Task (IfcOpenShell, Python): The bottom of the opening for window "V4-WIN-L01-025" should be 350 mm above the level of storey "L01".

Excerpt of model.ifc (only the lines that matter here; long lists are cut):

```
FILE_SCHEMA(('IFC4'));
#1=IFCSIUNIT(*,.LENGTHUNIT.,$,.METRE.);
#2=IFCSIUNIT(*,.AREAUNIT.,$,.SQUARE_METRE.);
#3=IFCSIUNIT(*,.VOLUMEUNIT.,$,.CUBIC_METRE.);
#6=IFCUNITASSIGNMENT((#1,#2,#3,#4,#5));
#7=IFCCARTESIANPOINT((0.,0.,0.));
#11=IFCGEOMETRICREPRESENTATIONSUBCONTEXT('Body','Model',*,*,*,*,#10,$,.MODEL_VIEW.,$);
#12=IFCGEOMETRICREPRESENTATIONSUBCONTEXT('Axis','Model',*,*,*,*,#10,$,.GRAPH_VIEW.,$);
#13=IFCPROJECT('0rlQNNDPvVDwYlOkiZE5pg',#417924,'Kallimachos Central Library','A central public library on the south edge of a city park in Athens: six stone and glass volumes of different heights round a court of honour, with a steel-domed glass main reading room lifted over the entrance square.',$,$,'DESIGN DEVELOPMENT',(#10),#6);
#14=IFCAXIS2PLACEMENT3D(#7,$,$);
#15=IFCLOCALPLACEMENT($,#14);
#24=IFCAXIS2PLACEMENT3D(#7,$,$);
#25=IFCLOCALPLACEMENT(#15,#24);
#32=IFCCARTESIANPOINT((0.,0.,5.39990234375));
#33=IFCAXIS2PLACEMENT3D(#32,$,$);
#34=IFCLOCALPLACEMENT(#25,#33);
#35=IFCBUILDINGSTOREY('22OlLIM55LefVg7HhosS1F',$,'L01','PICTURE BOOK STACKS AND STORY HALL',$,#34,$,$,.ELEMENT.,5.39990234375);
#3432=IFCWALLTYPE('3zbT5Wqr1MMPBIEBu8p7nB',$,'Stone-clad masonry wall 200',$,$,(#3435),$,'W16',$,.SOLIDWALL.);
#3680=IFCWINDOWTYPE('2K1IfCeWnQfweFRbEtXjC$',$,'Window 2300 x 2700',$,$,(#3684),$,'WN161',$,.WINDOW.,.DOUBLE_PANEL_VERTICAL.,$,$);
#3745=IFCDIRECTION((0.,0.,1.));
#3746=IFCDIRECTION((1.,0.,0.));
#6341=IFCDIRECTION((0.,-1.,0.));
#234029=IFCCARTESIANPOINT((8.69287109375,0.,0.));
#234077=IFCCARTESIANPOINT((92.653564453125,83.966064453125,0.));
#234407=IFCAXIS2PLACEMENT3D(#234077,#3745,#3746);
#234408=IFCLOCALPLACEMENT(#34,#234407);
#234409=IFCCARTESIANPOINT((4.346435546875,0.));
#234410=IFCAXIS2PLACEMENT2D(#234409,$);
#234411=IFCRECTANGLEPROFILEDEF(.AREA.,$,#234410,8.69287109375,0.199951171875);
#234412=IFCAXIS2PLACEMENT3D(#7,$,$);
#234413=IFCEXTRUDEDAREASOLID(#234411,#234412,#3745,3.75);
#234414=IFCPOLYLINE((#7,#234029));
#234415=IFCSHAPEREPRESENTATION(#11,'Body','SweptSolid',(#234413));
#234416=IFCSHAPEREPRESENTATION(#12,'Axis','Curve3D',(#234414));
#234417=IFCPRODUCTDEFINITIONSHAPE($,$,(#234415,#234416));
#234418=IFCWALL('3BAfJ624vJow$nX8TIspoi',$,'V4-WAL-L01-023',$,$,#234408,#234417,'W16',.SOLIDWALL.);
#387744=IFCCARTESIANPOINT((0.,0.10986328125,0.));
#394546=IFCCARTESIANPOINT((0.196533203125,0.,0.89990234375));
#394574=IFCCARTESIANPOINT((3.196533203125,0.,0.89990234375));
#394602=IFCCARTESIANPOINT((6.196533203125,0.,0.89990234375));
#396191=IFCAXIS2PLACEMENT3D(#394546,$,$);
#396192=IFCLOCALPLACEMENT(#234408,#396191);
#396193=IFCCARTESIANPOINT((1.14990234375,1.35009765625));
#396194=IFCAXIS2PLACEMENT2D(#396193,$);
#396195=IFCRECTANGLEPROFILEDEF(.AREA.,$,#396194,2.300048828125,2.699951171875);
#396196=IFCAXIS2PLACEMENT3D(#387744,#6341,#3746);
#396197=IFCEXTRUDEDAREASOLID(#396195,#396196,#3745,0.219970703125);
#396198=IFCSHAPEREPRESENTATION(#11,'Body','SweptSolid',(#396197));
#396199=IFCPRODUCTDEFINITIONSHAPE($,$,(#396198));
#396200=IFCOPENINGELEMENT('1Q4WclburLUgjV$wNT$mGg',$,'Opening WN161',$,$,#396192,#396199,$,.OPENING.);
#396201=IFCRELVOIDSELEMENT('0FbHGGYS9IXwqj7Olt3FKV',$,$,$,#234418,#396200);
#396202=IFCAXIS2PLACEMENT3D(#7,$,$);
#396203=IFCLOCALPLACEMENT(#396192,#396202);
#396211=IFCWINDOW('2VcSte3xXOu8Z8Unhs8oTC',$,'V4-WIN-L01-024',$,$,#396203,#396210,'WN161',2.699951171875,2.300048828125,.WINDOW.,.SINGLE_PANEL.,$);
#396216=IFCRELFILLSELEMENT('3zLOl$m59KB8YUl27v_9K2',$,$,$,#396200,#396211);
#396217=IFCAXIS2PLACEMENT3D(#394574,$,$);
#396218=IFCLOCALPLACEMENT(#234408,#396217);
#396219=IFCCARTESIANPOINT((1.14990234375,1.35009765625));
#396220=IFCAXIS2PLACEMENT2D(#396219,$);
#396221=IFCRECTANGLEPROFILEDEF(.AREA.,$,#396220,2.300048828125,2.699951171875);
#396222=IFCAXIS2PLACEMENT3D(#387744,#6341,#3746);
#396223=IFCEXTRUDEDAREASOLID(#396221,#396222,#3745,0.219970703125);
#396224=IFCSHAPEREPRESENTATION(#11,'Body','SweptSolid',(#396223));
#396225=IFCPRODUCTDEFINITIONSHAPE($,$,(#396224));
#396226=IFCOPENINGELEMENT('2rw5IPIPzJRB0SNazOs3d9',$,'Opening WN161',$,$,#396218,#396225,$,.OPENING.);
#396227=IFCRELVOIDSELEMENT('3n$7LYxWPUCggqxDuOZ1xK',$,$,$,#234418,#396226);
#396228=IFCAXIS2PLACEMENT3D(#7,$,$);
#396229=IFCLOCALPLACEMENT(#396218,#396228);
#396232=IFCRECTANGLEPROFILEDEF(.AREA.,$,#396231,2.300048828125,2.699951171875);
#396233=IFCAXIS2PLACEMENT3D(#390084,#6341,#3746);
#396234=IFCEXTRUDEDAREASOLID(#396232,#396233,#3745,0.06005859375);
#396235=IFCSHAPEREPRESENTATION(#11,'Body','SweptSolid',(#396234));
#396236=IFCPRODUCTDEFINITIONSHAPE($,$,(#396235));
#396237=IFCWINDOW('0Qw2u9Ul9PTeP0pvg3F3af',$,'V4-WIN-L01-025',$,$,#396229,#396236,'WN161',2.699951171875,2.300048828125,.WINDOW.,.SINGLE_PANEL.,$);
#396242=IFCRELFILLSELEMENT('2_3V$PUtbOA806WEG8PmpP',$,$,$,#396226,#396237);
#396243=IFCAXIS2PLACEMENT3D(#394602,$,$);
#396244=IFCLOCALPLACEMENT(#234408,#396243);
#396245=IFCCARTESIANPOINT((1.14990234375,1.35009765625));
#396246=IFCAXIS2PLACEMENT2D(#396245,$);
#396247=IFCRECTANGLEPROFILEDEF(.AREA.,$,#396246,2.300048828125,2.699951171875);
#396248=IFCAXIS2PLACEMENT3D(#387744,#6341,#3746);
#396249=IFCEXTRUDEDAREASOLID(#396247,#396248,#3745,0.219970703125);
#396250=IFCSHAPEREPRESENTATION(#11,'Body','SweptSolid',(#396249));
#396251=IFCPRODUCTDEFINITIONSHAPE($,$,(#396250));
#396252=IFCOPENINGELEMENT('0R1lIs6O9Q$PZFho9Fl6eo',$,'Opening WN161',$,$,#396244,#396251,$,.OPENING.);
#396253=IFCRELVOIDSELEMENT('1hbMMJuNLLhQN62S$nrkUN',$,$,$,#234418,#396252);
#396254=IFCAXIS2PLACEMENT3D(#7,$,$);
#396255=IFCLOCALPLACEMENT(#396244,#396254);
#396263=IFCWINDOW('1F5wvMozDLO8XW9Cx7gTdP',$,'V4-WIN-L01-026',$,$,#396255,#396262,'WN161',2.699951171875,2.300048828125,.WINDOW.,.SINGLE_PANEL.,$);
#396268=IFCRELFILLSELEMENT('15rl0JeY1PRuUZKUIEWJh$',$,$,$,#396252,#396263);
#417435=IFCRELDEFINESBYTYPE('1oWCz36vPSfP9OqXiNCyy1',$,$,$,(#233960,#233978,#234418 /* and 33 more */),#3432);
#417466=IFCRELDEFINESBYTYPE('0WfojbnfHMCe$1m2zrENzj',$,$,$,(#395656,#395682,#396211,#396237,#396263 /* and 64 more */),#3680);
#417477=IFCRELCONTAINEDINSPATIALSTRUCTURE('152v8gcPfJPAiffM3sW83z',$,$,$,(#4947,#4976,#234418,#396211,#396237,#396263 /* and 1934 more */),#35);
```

```python
import numpy as np
import ifcopenshell
import ifcopenshell.api.geometry
import ifcopenshell.geom
import ifcopenshell.util.element
import ifcopenshell.util.placement
import ifcopenshell.util.shape
import ifcopenshell.util.unit

model = ifcopenshell.open("model.ifc")
unit_scale = ifcopenshell.util.unit.calculate_unit_scale(model)

window = model.by_guid("0Qw2u9Ul9PTeP0pvg3F3af")
opening = window.FillsVoids[0].RelatingOpeningElement
storey = ifcopenshell.util.element.get_container(window, ifc_class="IfcBuildingStorey")
level = ifcopenshell.util.placement.get_local_placement(storey.ObjectPlacement)[2, 3]

# The opening's origin need not be at the sill, so measure its lowest point.
shape = ifcopenshell.geom.create_shape(ifcopenshell.geom.settings(), opening)
bottom = ifcopenshell.util.shape.get_shape_bottom_elevation(shape, shape.geometry) / unit_scale
dz = level + 0.35 - bottom

shift = np.array([0.0, 0.0, dz])
# The window is placed relative to its opening, so it follows when the opening moves.
matrix = ifcopenshell.util.placement.get_local_placement(opening.ObjectPlacement)
matrix[:3, 3] += shift
ifcopenshell.api.geometry.edit_object_placement(
    model, product=opening, matrix=matrix, is_si=False, should_transform_children=True
)

print(f"moved by {dz * unit_scale:+.3f} m")

model.write("model_edited.ifc")
```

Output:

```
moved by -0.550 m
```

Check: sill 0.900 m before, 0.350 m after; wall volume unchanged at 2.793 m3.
